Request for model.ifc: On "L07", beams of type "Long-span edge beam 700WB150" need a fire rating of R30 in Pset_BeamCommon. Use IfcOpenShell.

First a look at what the model holds.

```python
import ifcopenshell
import ifcopenshell.util.element

model = ifcopenshell.open("model.ifc")
print(model.schema)
storey = next(s for s in model.by_type("IfcBuildingStorey") if s.Name == "L07")
beams = [e for e in ifcopenshell.util.element.get_decomposition(storey) if e.is_a("IfcBeam")]
seen = {}
for e in beams:
    element_type = ifcopenshell.util.element.get_type(e)
    key = (element_type.Name if element_type != e and element_type else None, ifcopenshell.util.element.get_pset(e, "Pset_BeamCommon", "FireRating"))
    seen[key] = seen.get(key, 0) + 1
for (name, value), count in sorted(seen.items(), key=str):
    print(count, "x", name, "|", value)
```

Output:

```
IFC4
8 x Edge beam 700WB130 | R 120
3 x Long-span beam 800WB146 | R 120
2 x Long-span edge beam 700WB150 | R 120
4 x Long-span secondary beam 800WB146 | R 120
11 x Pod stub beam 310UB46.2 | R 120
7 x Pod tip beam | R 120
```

```python
import ifcopenshell
import ifcopenshell.api.pset
import ifcopenshell.util.element

model = ifcopenshell.open("model.ifc")

storey = next(s for s in model.by_type("IfcBuildingStorey") if s.Name == "L07")
beams = [e for e in ifcopenshell.util.element.get_decomposition(storey) if e.is_a("IfcBeam")]

count = 0
for e in beams:
    element_type = ifcopenshell.util.element.get_type(e)
    if element_type in (None, e) or element_type.Name != "Long-span edge beam 700WB150":
        continue
    # add_pset returns the element's existing set when there is one.
    pset = ifcopenshell.api.pset.add_pset(model, product=e, name="Pset_BeamCommon")
    ifcopenshell.api.pset.edit_pset(model, pset=pset, properties={"FireRating": "R30"})
    count += 1

print(count, "beams updated")

model.write("model_edited.ifc")
```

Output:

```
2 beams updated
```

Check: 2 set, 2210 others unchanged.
